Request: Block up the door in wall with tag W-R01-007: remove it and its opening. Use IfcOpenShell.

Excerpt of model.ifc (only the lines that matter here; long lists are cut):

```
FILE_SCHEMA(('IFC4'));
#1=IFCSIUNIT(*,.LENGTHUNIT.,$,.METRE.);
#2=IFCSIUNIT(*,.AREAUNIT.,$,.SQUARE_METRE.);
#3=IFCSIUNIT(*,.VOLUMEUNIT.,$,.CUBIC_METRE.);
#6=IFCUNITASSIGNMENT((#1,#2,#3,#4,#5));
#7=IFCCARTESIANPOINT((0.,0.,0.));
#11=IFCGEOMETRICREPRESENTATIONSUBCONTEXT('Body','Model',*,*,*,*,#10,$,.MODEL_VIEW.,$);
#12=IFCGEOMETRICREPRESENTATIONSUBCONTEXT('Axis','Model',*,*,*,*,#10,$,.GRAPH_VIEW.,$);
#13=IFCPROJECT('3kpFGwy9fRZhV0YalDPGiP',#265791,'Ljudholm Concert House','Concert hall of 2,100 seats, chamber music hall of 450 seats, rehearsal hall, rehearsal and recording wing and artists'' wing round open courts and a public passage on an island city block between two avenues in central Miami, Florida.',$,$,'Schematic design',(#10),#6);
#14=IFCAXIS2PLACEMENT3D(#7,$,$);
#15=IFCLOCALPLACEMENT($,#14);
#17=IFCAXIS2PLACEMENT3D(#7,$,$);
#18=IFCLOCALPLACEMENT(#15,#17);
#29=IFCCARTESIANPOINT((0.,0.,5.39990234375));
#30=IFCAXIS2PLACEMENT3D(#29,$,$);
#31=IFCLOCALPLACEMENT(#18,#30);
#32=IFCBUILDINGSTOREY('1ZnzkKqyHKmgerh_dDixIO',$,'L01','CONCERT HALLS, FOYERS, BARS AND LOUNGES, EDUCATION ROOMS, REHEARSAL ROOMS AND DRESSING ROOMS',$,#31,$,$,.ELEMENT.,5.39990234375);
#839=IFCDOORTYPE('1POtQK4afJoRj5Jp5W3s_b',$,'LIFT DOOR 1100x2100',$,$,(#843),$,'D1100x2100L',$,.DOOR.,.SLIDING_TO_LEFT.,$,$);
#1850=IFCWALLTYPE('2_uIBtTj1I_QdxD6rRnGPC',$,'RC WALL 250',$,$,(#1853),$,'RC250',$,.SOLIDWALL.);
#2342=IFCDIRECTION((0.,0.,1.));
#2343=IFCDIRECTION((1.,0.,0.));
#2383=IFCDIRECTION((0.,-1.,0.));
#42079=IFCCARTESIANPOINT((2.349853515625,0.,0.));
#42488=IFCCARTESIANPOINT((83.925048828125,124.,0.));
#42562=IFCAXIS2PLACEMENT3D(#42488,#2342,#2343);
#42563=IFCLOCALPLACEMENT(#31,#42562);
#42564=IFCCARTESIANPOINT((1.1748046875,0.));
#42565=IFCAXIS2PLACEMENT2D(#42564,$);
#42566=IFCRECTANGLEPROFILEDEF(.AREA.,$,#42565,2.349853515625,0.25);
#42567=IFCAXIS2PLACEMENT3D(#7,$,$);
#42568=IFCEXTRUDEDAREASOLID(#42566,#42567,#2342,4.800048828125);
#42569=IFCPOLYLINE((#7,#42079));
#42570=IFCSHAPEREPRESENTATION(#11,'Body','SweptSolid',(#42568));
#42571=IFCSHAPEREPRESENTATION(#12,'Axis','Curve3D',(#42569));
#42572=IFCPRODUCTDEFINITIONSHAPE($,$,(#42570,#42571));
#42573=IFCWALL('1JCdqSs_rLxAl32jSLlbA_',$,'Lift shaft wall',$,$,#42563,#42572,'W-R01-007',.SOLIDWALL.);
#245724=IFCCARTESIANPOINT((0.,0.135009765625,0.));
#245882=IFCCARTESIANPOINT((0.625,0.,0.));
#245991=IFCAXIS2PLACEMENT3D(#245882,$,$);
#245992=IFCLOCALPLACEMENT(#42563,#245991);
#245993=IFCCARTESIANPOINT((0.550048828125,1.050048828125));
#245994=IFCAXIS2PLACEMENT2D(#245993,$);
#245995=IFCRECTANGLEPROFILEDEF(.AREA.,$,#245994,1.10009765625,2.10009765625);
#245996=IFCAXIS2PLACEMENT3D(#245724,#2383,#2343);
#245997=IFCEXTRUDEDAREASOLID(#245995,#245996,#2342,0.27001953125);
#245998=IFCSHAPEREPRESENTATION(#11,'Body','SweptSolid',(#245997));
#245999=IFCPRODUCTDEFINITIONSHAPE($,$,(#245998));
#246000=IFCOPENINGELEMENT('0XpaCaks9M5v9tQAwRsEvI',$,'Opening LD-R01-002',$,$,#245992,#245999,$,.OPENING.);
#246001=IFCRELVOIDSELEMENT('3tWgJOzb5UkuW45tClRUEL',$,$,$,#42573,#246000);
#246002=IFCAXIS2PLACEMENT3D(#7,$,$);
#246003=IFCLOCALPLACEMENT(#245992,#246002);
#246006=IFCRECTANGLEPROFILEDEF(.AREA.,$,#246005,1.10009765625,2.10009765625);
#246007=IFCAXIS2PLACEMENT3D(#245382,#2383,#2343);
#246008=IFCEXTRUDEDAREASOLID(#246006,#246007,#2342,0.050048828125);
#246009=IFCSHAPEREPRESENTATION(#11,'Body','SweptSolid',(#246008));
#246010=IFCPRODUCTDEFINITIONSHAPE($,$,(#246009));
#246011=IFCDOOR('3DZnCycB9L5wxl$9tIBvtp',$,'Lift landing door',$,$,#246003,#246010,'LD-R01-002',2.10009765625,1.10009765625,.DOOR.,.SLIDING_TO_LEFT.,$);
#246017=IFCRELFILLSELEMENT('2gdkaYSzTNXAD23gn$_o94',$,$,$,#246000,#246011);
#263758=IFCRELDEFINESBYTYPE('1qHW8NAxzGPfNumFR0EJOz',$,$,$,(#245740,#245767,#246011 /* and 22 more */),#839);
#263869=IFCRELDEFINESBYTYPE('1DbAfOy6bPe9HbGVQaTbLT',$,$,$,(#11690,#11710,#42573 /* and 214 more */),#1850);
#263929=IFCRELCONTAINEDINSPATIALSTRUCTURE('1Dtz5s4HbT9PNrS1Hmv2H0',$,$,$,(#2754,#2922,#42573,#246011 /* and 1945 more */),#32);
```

```python
import ifcopenshell
import ifcopenshell.api.feature
import ifcopenshell.api.root
import ifcopenshell.geom
import ifcopenshell.util.shape

model = ifcopenshell.open("model.ifc")
settings = ifcopenshell.geom.settings()


def volume(element):
    """Net volume in cubic metres, openings subtracted."""
    shape = ifcopenshell.geom.create_shape(settings, element)
    return ifcopenshell.util.shape.get_volume(shape.geometry)


door = model.by_guid("3DZnCycB9L5wxl$9tIBvtp")
opening = door.FillsVoids[0].RelatingOpeningElement
wall = opening.VoidsElements[0].RelatingBuildingElement
before = volume(wall)

ifcopenshell.api.root.remove_product(model, product=door)
ifcopenshell.api.feature.remove_feature(model, feature=opening)

after = volume(wall)

print(f"wall volume {before:.3f} -> {after:.3f} m3")

model.write("model_rev.ifc")
```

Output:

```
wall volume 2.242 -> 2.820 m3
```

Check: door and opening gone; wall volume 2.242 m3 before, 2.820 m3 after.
